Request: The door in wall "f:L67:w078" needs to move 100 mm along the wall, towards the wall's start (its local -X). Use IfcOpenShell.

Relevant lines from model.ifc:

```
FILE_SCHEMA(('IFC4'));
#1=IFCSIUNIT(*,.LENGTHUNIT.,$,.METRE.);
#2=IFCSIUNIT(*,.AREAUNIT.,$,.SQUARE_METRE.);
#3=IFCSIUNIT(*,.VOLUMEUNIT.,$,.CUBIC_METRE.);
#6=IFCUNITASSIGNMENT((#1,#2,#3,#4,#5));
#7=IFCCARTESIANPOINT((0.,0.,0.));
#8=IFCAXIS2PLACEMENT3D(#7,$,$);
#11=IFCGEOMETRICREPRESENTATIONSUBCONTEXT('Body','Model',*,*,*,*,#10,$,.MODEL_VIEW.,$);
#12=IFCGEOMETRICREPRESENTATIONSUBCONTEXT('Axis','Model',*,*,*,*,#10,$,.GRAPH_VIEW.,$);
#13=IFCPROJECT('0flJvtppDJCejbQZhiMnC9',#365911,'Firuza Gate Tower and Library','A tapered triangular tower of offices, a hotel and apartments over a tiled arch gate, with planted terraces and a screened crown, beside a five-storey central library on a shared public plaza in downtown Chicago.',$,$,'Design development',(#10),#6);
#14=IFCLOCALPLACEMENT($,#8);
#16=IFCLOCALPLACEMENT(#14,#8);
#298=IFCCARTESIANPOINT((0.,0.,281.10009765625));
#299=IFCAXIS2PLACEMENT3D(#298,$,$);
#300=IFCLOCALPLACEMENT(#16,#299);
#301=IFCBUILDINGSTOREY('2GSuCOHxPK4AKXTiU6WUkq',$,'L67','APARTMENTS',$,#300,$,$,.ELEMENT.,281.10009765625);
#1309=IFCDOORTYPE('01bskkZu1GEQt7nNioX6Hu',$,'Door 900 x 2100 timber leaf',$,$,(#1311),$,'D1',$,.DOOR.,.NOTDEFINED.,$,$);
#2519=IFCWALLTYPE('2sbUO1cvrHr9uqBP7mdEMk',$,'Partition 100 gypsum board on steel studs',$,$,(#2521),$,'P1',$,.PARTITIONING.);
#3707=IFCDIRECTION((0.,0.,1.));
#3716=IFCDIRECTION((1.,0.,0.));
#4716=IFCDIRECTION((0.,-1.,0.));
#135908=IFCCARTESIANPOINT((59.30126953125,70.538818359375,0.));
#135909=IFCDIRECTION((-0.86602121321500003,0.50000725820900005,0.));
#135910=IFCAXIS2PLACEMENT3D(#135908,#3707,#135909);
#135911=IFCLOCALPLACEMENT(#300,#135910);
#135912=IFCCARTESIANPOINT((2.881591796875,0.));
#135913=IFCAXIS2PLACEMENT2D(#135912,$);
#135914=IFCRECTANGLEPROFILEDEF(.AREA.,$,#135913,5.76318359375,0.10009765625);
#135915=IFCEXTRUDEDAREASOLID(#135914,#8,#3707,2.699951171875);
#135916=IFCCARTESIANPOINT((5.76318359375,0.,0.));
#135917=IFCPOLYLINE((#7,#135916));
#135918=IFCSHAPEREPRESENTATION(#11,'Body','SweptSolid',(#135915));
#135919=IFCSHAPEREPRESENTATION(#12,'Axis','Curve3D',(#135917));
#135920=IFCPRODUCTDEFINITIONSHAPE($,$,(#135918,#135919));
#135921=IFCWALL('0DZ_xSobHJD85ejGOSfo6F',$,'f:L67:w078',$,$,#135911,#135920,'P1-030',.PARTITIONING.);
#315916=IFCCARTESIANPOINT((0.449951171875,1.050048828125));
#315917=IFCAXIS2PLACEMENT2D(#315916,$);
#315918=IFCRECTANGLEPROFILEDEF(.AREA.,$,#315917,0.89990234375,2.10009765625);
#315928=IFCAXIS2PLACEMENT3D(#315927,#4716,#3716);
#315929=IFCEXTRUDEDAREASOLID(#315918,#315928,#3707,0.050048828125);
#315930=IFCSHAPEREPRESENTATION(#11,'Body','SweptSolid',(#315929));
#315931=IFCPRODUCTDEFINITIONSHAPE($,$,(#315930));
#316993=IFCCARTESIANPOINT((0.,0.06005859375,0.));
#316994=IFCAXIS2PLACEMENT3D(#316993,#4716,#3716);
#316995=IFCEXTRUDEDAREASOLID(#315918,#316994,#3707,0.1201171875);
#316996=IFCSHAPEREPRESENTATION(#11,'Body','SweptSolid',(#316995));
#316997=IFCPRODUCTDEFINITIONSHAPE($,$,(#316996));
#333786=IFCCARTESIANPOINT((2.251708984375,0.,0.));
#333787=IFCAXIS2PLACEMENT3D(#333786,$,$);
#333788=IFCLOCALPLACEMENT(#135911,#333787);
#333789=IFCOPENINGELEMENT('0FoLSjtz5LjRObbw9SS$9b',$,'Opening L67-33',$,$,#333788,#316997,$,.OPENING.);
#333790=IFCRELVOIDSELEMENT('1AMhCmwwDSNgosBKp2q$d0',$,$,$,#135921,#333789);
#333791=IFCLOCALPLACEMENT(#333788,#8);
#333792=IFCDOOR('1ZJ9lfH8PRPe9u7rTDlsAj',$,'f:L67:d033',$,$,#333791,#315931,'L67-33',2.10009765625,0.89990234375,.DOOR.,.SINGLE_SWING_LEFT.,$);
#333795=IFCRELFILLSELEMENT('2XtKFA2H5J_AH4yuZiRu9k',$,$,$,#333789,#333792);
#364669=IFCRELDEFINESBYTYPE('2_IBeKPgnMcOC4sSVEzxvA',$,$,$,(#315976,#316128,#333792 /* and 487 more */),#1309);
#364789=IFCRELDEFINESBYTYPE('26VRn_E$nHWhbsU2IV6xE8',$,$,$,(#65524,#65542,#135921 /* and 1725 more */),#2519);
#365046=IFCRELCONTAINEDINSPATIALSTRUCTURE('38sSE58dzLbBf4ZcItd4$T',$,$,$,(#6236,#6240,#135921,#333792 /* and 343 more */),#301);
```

```python
import ifcopenshell
import ifcopenshell.api.geometry
import ifcopenshell.util.placement
import ifcopenshell.util.unit

model = ifcopenshell.open("model.ifc")
unit_scale = ifcopenshell.util.unit.calculate_unit_scale(model)

door = model.by_guid("1ZJ9lfH8PRPe9u7rTDlsAj")
opening = door.FillsVoids[0].RelatingOpeningElement
wall = opening.VoidsElements[0].RelatingBuildingElement

wall_matrix = ifcopenshell.util.placement.get_local_placement(wall.ObjectPlacement)
shift = wall_matrix[:3, 0] * -0.1 / unit_scale
before = ifcopenshell.util.placement.get_local_placement(door.ObjectPlacement)[:3, 3].copy()

# The door is placed relative to its opening, so it follows when the opening moves.
matrix = ifcopenshell.util.placement.get_local_placement(opening.ObjectPlacement)
matrix[:3, 3] += shift
ifcopenshell.api.geometry.edit_object_placement(
    model, product=opening, matrix=matrix, is_si=False, should_transform_children=True
)

after = ifcopenshell.util.placement.get_local_placement(door.ObjectPlacement)[:3, 3]
print("door moved by", (after - before).round(3) + 0.0)

model.write("model_v2.ifc")
```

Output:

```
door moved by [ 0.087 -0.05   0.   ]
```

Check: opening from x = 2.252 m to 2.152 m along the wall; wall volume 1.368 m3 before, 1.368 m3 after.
